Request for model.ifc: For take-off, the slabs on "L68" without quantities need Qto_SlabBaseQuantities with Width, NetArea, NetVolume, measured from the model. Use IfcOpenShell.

First a look at what the model holds.

```python
import ifcopenshell
import ifcopenshell.util.element
import ifcopenshell.util.unit

model = ifcopenshell.open("model.ifc")
print(model.schema)
for unit_type in ("LENGTHUNIT", "AREAUNIT", "VOLUMEUNIT"):
    print(unit_type, ifcopenshell.util.unit.calculate_unit_scale(model, unit_type))
storey = next(s for s in model.by_type("IfcBuildingStorey") if s.Name == "L68")
slabs = [e for e in ifcopenshell.util.element.get_decomposition(storey) if e.is_a("IfcSlab")]
for e in sorted(slabs, key=lambda e: e.id()):
    print(e.id(), e.is_a(), e.Name, list(ifcopenshell.util.element.get_psets(e, qtos_only=True)), sep=" | ")
```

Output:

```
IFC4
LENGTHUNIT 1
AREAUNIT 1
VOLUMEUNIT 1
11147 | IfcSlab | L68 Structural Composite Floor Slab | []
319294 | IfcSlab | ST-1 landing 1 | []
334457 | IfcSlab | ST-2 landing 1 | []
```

```python
import ifcopenshell
import ifcopenshell.api.pset
import ifcopenshell.geom
import ifcopenshell.util.element
import ifcopenshell.util.shape
import ifcopenshell.util.unit

model = ifcopenshell.open("model.ifc")
unit_scale = ifcopenshell.util.unit.calculate_unit_scale(model)
area_scale = ifcopenshell.util.unit.calculate_unit_scale(model, "AREAUNIT")
volume_scale = ifcopenshell.util.unit.calculate_unit_scale(model, "VOLUMEUNIT")
settings = ifcopenshell.geom.settings()

storey = next(s for s in model.by_type("IfcBuildingStorey") if s.Name == "L68")
slabs = [e for e in ifcopenshell.util.element.get_decomposition(storey) if e.is_a("IfcSlab")]

for e in sorted(slabs, key=lambda e: e.id()):
    if ifcopenshell.util.element.get_psets(e, qtos_only=True, should_inherit=False):
        continue
    # Geometry comes back in metres, in the element's own axes.
    shape = ifcopenshell.geom.create_shape(settings, e)
    values = {
        "Width": ifcopenshell.util.shape.get_z(shape.geometry) / unit_scale,
        "NetArea": ifcopenshell.util.shape.get_footprint_area(shape.geometry) / area_scale,
        "NetVolume": ifcopenshell.util.shape.get_volume(shape.geometry) / volume_scale,
    }
    qto = ifcopenshell.api.pset.add_qto(model, product=e, name="Qto_SlabBaseQuantities")
    ifcopenshell.api.pset.edit_qto(model, qto=qto, properties=values)
    print(e.id(), {k: round(v, 3) for k, v in values.items()})

model.write("model-out.ifc")
```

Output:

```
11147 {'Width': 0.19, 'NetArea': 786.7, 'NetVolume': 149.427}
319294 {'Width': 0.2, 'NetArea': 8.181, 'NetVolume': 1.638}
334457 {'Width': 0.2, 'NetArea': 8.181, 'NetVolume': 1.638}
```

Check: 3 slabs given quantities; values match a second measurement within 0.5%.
